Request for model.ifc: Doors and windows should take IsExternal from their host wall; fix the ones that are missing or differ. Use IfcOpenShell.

First a look at what the model holds.

```python
import ifcopenshell
import ifcopenshell.util.element

model = ifcopenshell.open("model.ifc")
print(model.schema)
seen = {}
for e in model.by_type("IfcDoor") + model.by_type("IfcWindow"):
    if not e.FillsVoids:
        continue
    host = e.FillsVoids[0].RelatingOpeningElement.VoidsElements[0].RelatingBuildingElement
    own = ifcopenshell.util.element.get_pset(e, f"Pset_{e.is_a()[3:].removesuffix('StandardCase')}Common", "IsExternal")
    wall = ifcopenshell.util.element.get_pset(host, "Pset_WallCommon", "IsExternal")
    seen[e.is_a(), own, wall] = seen.get((e.is_a(), own, wall), 0) + 1
for (cls, own, wall), count in sorted(seen.items(), key=str):
    print(count, cls, "IsExternal:", own, "| host wall:", wall)
```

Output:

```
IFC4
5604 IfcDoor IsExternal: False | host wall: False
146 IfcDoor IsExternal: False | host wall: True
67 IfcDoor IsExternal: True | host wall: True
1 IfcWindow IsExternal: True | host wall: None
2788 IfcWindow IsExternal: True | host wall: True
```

```python
import ifcopenshell
import ifcopenshell.api.pset
import ifcopenshell.util.element

model = ifcopenshell.open("model.ifc")

count = 0
for ifc_class, pset_name in (("IfcDoor", "Pset_DoorCommon"), ("IfcWindow", "Pset_WindowCommon")):
    for e in model.by_type(ifc_class):
        if not e.FillsVoids:
            continue
        host = e.FillsVoids[0].RelatingOpeningElement.VoidsElements[0].RelatingBuildingElement
        external = ifcopenshell.util.element.get_pset(host, "Pset_WallCommon", "IsExternal")
        if external is None or ifcopenshell.util.element.get_pset(e, pset_name, "IsExternal") == external:
            continue
        found = ifcopenshell.util.element.get_pset(e, pset_name, should_inherit=False)
        if found:
            pset = model.by_id(found["id"])
            if len(ifcopenshell.util.element.get_elements_by_pset(pset)) > 1:
                pset = ifcopenshell.api.pset.unshare_pset(model, products=[e], pset=pset)[0]
        else:
            pset = ifcopenshell.api.pset.add_pset(model, product=e, name=pset_name)
        ifcopenshell.api.pset.edit_pset(model, pset=pset, properties={"IsExternal": external})
        count += 1

print(count, "updated")

model.write("model-out.ifc")
```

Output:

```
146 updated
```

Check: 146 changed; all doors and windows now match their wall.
